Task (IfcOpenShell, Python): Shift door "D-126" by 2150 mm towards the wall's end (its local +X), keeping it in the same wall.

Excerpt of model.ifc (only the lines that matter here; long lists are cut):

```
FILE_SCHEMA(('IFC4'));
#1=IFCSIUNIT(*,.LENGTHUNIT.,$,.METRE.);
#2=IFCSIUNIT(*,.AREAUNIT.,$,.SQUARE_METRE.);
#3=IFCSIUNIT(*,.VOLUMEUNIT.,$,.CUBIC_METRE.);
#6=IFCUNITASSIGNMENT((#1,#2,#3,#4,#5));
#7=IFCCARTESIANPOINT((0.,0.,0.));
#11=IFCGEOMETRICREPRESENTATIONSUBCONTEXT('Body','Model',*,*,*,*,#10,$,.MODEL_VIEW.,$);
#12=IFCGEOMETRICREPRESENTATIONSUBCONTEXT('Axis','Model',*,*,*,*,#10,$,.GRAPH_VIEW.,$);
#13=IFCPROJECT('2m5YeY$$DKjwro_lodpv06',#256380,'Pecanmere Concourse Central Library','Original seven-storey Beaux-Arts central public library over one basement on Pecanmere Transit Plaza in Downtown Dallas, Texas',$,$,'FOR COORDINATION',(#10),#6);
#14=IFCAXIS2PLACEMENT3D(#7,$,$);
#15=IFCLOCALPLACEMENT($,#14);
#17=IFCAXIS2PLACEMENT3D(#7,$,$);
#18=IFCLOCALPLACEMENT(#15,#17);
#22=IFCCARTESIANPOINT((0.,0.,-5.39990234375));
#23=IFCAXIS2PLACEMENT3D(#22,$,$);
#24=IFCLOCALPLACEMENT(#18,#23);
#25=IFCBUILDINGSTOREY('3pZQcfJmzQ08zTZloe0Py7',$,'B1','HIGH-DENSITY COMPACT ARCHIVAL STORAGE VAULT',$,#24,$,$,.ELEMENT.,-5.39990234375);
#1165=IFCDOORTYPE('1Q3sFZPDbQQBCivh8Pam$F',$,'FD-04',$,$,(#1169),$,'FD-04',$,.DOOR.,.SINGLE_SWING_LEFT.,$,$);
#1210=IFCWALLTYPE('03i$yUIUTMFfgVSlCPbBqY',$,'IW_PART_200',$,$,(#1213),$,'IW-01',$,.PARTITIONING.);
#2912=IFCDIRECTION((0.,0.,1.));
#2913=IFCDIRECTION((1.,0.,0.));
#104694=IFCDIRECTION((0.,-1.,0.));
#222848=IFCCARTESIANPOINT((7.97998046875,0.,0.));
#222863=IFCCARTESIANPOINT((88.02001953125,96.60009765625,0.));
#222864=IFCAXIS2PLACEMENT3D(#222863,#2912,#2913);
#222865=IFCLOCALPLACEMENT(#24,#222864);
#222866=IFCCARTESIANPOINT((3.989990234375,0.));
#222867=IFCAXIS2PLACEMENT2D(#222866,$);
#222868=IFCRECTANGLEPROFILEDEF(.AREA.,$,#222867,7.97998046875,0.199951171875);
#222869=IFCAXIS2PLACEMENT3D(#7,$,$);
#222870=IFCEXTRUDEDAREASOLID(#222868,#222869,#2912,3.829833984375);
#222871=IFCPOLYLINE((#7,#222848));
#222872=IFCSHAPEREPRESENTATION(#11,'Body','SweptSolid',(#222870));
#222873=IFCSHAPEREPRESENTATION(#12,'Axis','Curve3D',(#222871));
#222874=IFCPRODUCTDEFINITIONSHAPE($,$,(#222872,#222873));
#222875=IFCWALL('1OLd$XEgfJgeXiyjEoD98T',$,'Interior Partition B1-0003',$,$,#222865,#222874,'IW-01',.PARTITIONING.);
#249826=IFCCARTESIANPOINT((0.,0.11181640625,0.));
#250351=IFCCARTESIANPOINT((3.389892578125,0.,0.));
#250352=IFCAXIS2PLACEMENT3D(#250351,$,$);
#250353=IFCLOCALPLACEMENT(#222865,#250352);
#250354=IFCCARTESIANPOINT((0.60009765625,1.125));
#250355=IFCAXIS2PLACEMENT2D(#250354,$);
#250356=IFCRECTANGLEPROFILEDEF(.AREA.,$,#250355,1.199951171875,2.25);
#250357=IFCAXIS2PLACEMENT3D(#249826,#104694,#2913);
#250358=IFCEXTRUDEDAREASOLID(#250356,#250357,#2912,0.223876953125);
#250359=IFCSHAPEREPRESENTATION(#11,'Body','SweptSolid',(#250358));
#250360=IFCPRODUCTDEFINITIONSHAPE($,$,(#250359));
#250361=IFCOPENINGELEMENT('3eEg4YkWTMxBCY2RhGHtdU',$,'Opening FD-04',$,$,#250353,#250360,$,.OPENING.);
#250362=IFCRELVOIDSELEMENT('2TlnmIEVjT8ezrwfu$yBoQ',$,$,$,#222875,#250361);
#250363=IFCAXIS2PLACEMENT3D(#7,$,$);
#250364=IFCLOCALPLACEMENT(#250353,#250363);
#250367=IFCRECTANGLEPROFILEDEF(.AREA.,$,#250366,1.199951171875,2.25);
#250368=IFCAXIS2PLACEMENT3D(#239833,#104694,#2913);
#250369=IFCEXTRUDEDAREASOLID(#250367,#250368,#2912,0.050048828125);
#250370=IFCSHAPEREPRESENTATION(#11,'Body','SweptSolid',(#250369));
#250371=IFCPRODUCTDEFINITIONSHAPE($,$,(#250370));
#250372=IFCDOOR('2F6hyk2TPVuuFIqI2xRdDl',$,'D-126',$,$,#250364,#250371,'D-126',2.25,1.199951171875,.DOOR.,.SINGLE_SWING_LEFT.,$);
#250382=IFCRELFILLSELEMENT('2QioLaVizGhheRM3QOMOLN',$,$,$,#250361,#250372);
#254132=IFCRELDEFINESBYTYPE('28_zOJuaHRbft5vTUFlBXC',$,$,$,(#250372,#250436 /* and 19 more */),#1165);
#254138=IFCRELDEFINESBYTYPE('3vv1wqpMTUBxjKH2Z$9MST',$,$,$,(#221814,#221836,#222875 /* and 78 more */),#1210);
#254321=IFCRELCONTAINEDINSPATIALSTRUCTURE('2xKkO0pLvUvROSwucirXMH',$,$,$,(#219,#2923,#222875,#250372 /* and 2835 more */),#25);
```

```python
import ifcopenshell
import ifcopenshell.api.geometry
import ifcopenshell.util.placement
import ifcopenshell.util.unit

model = ifcopenshell.open("model.ifc")
unit_scale = ifcopenshell.util.unit.calculate_unit_scale(model)

door = model.by_guid("2F6hyk2TPVuuFIqI2xRdDl")
opening = door.FillsVoids[0].RelatingOpeningElement
wall = opening.VoidsElements[0].RelatingBuildingElement

wall_matrix = ifcopenshell.util.placement.get_local_placement(wall.ObjectPlacement)
shift = wall_matrix[:3, 0] * 2.15 / unit_scale
before = ifcopenshell.util.placement.get_local_placement(door.ObjectPlacement)[:3, 3].copy()

# The door is placed relative to its opening, so it follows when the opening moves.
matrix = ifcopenshell.util.placement.get_local_placement(opening.ObjectPlacement)
matrix[:3, 3] += shift
ifcopenshell.api.geometry.edit_object_placement(
    model, product=opening, matrix=matrix, is_si=False, should_transform_children=True
)

after = ifcopenshell.util.placement.get_local_placement(door.ObjectPlacement)[:3, 3]
print("door moved by", (after - before).round(3) + 0.0)

model.write("model_edited.ifc")
```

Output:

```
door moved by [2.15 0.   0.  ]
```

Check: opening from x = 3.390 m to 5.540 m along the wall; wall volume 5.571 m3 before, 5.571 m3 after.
